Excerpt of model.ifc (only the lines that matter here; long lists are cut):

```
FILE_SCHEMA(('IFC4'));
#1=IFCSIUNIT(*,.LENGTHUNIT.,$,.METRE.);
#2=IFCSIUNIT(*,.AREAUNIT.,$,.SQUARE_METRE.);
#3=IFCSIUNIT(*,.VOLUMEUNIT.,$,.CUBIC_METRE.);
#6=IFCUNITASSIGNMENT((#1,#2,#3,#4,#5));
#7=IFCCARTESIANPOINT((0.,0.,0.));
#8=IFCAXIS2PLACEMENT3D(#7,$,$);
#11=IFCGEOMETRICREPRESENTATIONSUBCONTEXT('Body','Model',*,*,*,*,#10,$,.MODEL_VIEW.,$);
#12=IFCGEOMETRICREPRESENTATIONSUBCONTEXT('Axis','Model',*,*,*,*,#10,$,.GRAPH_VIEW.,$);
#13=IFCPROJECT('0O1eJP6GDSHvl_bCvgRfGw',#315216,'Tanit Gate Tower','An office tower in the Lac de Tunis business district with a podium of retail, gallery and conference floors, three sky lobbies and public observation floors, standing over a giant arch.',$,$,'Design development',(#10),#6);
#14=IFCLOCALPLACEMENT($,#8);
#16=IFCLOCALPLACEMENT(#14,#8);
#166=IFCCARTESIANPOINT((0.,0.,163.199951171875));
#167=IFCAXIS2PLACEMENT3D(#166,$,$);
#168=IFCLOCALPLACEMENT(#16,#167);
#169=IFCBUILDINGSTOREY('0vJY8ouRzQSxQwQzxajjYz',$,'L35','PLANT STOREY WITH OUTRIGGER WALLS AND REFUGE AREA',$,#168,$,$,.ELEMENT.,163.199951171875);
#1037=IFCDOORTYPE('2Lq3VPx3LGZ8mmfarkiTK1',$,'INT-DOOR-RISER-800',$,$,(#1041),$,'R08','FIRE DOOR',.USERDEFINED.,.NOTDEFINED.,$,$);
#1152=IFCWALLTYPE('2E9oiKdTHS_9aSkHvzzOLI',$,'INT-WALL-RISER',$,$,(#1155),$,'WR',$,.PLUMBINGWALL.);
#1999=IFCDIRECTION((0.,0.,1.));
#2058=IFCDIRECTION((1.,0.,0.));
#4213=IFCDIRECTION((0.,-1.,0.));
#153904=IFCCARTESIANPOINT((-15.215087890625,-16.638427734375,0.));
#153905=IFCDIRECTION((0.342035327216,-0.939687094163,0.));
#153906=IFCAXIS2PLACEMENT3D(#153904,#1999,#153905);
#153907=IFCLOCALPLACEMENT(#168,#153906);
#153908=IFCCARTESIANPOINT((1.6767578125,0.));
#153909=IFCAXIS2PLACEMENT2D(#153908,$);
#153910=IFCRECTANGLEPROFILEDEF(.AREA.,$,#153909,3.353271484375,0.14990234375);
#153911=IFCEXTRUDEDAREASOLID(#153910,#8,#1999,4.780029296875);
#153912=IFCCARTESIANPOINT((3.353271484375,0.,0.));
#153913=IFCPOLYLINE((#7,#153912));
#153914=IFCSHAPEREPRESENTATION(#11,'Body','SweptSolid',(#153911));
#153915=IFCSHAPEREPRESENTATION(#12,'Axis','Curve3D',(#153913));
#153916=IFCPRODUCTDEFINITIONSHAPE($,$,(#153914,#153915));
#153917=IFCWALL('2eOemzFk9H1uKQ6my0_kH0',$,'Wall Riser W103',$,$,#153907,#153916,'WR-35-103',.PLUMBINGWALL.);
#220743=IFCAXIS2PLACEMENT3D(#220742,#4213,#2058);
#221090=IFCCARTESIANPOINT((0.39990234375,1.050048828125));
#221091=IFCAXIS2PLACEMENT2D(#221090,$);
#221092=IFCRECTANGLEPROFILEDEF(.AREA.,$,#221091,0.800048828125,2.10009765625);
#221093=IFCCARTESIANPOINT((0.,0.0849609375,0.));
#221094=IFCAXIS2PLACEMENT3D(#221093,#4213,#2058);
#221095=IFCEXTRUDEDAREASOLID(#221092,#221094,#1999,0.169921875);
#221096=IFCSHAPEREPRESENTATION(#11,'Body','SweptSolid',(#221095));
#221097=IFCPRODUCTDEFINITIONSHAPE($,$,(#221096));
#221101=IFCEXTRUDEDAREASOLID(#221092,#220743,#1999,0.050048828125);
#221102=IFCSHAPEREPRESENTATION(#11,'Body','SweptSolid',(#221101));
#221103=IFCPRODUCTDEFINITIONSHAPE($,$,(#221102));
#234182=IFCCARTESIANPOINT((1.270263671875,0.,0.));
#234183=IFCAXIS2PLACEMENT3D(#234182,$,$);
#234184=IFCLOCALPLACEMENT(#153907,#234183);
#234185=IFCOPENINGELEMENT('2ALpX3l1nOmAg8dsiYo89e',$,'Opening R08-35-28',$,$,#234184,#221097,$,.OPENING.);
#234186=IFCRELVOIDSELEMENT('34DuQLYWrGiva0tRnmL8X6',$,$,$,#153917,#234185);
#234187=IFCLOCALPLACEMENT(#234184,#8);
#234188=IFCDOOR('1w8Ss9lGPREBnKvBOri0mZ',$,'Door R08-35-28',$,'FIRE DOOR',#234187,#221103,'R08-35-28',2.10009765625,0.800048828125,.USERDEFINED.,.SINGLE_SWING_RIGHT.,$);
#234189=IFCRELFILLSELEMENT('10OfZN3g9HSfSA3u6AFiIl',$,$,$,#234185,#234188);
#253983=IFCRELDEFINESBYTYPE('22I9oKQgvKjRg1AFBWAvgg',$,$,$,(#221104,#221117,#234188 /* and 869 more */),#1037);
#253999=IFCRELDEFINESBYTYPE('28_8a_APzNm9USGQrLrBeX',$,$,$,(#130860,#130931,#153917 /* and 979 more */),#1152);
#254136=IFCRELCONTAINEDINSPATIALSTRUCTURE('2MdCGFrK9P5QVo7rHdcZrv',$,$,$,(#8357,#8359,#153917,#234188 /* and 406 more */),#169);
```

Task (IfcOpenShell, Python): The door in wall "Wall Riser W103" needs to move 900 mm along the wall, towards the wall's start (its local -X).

```python
import ifcopenshell
import ifcopenshell.api.geometry
import ifcopenshell.util.placement

model = ifcopenshell.open("model.ifc")

door = model.by_guid("1w8Ss9lGPREBnKvBOri0mZ")
opening = door.FillsVoids[0].RelatingOpeningElement
wall = opening.VoidsElements[0].RelatingBuildingElement

wall_matrix = ifcopenshell.util.placement.get_local_placement(wall.ObjectPlacement)
shift = wall_matrix[:3, 0] * -0.9
before = ifcopenshell.util.placement.get_local_placement(door.ObjectPlacement)[:3, 3].copy()

# The door is placed relative to its opening, so it follows when the opening moves.
matrix = ifcopenshell.util.placement.get_local_placement(opening.ObjectPlacement)
matrix[:3, 3] += shift
ifcopenshell.api.geometry.edit_object_placement(
    model, product=opening, matrix=matrix, is_si=False, should_transform_children=True
)

after = ifcopenshell.util.placement.get_local_placement(door.ObjectPlacement)[:3, 3]
print("door moved by", (after - before).round(3) + 0.0)

model.write("model_rev.ifc")
```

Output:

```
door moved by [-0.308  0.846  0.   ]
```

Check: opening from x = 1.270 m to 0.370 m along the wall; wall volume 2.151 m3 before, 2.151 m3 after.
